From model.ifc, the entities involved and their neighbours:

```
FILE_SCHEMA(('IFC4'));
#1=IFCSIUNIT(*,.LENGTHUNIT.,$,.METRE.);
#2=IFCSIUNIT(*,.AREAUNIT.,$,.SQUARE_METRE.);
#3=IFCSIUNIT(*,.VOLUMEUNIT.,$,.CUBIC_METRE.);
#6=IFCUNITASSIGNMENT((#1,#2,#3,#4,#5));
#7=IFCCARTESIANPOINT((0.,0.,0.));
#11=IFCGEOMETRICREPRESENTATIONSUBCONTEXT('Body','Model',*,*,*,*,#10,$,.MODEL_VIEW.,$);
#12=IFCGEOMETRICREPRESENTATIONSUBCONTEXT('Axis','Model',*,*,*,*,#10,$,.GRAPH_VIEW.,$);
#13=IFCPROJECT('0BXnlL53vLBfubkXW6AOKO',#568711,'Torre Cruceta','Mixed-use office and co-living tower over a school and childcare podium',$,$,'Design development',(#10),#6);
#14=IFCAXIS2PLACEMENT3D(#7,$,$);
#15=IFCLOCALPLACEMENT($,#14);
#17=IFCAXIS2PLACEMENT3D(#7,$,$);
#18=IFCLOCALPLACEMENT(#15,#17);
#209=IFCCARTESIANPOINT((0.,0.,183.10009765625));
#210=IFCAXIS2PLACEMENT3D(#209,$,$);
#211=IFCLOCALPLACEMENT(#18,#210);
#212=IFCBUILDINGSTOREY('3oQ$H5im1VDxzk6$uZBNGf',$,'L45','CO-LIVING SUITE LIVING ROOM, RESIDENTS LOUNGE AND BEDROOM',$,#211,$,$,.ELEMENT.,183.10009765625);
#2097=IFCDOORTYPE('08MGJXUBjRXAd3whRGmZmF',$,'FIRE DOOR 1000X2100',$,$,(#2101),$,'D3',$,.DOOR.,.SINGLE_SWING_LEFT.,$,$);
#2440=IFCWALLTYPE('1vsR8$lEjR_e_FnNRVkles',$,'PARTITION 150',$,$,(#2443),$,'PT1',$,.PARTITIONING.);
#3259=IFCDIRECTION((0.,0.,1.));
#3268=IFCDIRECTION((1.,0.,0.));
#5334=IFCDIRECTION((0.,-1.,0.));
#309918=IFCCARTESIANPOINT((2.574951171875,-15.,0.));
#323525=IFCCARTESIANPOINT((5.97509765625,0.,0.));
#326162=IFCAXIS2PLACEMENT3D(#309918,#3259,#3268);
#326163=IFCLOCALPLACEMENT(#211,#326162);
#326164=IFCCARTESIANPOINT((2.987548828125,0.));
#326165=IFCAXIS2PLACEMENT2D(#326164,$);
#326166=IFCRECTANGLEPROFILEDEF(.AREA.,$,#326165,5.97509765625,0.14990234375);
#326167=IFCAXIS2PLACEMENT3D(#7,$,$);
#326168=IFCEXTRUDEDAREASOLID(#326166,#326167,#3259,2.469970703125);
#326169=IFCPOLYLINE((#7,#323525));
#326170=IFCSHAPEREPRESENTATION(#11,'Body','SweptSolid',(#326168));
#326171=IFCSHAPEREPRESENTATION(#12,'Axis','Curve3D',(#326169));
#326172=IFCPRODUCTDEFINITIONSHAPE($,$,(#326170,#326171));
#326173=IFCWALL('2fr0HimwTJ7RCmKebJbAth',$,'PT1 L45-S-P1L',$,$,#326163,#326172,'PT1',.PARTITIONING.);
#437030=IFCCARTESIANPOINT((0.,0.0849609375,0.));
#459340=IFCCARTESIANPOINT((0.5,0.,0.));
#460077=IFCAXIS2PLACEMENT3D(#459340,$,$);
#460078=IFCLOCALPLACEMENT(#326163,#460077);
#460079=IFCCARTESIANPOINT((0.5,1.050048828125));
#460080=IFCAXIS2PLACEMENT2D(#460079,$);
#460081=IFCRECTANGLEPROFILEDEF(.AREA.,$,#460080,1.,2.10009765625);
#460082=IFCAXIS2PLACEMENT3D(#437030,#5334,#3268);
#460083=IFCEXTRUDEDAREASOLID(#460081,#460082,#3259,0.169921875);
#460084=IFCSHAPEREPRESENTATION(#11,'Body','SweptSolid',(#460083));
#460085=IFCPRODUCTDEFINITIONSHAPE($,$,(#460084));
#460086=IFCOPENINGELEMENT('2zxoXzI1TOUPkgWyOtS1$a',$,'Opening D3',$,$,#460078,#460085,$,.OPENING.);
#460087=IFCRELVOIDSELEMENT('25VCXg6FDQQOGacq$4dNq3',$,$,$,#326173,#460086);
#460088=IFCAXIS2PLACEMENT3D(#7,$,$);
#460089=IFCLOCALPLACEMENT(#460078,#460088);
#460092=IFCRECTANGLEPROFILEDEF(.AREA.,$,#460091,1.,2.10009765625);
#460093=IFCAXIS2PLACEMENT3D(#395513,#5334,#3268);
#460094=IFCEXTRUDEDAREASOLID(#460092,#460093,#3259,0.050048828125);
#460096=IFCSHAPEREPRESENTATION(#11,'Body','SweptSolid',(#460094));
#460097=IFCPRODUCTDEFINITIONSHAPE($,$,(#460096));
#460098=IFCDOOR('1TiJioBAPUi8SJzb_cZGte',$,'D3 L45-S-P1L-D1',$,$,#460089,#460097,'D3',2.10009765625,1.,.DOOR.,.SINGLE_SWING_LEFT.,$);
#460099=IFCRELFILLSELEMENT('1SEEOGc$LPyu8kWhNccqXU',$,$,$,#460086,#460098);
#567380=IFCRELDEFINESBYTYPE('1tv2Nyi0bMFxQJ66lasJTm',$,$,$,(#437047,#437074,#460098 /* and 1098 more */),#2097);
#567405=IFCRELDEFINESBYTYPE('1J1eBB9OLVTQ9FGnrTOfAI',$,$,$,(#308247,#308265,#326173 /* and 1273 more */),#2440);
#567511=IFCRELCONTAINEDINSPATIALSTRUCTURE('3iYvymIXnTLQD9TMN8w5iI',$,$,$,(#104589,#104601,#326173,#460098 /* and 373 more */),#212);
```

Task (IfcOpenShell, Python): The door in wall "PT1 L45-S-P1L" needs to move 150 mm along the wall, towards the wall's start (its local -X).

```python
import ifcopenshell
import ifcopenshell.api.geometry
import ifcopenshell.util.placement
import ifcopenshell.util.unit

model = ifcopenshell.open("model.ifc")
unit_scale = ifcopenshell.util.unit.calculate_unit_scale(model)

door = model.by_guid("1TiJioBAPUi8SJzb_cZGte")
opening = door.FillsVoids[0].RelatingOpeningElement
wall = opening.VoidsElements[0].RelatingBuildingElement

wall_matrix = ifcopenshell.util.placement.get_local_placement(wall.ObjectPlacement)
shift = wall_matrix[:3, 0] * -0.15 / unit_scale
before = ifcopenshell.util.placement.get_local_placement(door.ObjectPlacement)[:3, 3].copy()

# The door is placed relative to its opening, so it follows when the opening moves.
matrix = ifcopenshell.util.placement.get_local_placement(opening.ObjectPlacement)
matrix[:3, 3] += shift
ifcopenshell.api.geometry.edit_object_placement(
    model, product=opening, matrix=matrix, is_si=False, should_transform_children=True
)

after = ifcopenshell.util.placement.get_local_placement(door.ObjectPlacement)[:3, 3]
print("door moved by", (after - before).round(3) + 0.0)

model.write("model_edited.ifc")
```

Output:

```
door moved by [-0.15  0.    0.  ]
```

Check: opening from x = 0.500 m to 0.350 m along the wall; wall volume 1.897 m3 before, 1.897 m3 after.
